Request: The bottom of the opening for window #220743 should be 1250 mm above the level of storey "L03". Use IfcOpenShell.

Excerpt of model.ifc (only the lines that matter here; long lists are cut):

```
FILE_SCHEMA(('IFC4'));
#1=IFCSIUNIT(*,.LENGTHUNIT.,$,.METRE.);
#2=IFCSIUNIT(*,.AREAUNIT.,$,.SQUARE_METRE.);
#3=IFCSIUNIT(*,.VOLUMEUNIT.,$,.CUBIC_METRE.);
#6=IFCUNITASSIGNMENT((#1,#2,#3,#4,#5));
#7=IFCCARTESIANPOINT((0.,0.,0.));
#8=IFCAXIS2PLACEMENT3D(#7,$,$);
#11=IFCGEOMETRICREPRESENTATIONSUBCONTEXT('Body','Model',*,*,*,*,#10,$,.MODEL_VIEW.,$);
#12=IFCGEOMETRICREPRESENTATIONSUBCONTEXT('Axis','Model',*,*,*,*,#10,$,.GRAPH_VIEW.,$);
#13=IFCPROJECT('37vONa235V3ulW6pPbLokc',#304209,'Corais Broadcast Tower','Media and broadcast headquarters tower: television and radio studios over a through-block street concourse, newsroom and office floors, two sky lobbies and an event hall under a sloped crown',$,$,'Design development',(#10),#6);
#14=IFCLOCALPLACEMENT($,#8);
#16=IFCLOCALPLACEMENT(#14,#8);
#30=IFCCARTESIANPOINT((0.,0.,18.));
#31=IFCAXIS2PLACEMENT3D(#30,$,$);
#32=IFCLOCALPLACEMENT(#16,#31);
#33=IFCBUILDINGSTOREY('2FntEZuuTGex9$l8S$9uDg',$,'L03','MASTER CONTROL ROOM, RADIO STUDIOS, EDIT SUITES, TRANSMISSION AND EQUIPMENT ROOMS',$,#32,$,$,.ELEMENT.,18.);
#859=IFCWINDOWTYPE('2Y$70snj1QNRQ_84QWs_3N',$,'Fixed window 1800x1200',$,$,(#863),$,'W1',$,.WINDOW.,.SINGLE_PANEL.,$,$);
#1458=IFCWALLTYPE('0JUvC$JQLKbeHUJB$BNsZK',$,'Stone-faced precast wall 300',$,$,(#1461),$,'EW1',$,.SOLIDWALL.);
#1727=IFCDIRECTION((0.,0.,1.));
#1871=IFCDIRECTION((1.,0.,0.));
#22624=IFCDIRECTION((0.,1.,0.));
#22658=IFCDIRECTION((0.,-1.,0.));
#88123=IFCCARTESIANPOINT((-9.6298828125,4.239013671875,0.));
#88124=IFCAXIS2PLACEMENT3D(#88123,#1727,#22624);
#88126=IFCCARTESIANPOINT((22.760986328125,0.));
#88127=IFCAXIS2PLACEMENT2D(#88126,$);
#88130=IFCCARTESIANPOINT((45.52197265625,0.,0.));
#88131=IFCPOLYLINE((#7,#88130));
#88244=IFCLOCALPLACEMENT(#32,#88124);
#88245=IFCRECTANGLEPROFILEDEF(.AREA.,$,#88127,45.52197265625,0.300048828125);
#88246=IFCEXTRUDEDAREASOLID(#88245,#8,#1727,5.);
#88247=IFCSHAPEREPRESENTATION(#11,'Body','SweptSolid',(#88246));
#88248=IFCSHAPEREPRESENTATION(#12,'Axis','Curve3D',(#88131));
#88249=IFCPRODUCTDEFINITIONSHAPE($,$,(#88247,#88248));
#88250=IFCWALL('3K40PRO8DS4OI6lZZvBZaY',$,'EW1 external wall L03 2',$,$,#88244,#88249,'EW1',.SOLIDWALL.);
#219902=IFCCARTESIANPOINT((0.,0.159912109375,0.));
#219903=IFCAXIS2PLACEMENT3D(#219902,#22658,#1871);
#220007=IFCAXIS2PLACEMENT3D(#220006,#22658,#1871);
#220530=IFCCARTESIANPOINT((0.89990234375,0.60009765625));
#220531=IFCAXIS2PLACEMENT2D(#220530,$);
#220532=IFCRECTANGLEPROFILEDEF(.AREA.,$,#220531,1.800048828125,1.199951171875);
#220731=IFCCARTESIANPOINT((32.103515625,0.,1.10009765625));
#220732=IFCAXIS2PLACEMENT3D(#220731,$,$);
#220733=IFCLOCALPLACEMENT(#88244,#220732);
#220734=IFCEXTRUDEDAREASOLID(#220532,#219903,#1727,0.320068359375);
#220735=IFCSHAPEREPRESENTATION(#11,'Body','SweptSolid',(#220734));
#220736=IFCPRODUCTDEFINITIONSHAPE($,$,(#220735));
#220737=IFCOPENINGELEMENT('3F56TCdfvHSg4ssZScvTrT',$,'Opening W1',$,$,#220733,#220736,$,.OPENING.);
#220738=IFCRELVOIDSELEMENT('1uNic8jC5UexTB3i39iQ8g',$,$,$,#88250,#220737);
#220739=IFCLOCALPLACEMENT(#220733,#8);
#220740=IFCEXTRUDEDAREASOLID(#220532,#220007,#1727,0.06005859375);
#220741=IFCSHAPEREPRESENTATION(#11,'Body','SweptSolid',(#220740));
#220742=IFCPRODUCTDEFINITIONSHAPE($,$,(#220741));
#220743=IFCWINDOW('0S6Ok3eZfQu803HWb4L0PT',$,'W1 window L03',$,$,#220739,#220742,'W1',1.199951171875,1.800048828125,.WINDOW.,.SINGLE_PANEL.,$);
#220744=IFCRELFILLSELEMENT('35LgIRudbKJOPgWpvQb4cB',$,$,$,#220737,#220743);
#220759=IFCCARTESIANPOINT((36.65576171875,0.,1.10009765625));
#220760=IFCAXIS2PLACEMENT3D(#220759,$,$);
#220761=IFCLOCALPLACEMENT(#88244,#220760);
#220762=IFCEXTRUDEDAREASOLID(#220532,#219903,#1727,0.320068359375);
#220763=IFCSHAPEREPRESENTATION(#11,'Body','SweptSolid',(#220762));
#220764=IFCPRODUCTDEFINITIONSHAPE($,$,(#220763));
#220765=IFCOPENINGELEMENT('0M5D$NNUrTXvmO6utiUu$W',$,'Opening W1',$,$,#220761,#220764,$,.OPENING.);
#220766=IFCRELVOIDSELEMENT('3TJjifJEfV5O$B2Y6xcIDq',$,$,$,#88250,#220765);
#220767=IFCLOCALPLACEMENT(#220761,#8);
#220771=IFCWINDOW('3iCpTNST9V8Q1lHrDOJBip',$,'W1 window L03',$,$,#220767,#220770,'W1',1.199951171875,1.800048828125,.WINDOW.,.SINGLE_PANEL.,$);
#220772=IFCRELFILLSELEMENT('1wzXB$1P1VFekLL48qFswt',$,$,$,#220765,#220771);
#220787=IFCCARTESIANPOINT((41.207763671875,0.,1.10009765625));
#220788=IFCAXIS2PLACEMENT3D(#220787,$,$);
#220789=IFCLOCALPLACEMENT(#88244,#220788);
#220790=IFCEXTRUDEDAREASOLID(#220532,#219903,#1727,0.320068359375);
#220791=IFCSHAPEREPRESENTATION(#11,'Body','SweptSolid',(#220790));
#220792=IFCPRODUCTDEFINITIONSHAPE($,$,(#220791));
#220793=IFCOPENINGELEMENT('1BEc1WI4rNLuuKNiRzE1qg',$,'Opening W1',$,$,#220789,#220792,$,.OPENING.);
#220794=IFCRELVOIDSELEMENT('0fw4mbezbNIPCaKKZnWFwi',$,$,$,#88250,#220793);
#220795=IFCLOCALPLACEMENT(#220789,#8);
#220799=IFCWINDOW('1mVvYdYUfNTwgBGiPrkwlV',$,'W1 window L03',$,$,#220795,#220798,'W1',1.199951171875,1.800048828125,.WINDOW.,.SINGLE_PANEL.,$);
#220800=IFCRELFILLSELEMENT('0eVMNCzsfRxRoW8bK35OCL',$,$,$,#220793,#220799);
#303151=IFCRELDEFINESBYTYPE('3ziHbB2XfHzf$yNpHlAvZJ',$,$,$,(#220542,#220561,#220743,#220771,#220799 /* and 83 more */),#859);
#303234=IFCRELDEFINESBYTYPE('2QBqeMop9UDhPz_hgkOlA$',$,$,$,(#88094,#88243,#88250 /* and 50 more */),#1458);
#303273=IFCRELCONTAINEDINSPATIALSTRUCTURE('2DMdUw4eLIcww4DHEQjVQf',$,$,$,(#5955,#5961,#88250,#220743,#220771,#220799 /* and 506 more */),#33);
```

```python
import numpy as np
import ifcopenshell
import ifcopenshell.api.geometry
import ifcopenshell.geom
import ifcopenshell.util.element
import ifcopenshell.util.placement
import ifcopenshell.util.shape
import ifcopenshell.util.unit

model = ifcopenshell.open("model.ifc")
unit_scale = ifcopenshell.util.unit.calculate_unit_scale(model)

window = model.by_guid("0S6Ok3eZfQu803HWb4L0PT")
opening = window.FillsVoids[0].RelatingOpeningElement
storey = ifcopenshell.util.element.get_container(window, ifc_class="IfcBuildingStorey")
level = ifcopenshell.util.placement.get_local_placement(storey.ObjectPlacement)[2, 3]

# The opening's origin need not be at the sill, so measure its lowest point.
shape = ifcopenshell.geom.create_shape(ifcopenshell.geom.settings(), opening)
bottom = ifcopenshell.util.shape.get_shape_bottom_elevation(shape, shape.geometry) / unit_scale
dz = level + 1.25 / unit_scale - bottom

shift = np.array([0.0, 0.0, dz])
# The window is placed relative to its opening, so it follows when the opening moves.
matrix = ifcopenshell.util.placement.get_local_placement(opening.ObjectPlacement)
matrix[:3, 3] += shift
ifcopenshell.api.geometry.edit_object_placement(
    model, product=opening, matrix=matrix, is_si=False, should_transform_children=True
)

print(f"moved by {dz * unit_scale:+.3f} m")

model.write("model_rev.ifc")
```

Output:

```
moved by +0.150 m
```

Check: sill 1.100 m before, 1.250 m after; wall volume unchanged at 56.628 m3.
